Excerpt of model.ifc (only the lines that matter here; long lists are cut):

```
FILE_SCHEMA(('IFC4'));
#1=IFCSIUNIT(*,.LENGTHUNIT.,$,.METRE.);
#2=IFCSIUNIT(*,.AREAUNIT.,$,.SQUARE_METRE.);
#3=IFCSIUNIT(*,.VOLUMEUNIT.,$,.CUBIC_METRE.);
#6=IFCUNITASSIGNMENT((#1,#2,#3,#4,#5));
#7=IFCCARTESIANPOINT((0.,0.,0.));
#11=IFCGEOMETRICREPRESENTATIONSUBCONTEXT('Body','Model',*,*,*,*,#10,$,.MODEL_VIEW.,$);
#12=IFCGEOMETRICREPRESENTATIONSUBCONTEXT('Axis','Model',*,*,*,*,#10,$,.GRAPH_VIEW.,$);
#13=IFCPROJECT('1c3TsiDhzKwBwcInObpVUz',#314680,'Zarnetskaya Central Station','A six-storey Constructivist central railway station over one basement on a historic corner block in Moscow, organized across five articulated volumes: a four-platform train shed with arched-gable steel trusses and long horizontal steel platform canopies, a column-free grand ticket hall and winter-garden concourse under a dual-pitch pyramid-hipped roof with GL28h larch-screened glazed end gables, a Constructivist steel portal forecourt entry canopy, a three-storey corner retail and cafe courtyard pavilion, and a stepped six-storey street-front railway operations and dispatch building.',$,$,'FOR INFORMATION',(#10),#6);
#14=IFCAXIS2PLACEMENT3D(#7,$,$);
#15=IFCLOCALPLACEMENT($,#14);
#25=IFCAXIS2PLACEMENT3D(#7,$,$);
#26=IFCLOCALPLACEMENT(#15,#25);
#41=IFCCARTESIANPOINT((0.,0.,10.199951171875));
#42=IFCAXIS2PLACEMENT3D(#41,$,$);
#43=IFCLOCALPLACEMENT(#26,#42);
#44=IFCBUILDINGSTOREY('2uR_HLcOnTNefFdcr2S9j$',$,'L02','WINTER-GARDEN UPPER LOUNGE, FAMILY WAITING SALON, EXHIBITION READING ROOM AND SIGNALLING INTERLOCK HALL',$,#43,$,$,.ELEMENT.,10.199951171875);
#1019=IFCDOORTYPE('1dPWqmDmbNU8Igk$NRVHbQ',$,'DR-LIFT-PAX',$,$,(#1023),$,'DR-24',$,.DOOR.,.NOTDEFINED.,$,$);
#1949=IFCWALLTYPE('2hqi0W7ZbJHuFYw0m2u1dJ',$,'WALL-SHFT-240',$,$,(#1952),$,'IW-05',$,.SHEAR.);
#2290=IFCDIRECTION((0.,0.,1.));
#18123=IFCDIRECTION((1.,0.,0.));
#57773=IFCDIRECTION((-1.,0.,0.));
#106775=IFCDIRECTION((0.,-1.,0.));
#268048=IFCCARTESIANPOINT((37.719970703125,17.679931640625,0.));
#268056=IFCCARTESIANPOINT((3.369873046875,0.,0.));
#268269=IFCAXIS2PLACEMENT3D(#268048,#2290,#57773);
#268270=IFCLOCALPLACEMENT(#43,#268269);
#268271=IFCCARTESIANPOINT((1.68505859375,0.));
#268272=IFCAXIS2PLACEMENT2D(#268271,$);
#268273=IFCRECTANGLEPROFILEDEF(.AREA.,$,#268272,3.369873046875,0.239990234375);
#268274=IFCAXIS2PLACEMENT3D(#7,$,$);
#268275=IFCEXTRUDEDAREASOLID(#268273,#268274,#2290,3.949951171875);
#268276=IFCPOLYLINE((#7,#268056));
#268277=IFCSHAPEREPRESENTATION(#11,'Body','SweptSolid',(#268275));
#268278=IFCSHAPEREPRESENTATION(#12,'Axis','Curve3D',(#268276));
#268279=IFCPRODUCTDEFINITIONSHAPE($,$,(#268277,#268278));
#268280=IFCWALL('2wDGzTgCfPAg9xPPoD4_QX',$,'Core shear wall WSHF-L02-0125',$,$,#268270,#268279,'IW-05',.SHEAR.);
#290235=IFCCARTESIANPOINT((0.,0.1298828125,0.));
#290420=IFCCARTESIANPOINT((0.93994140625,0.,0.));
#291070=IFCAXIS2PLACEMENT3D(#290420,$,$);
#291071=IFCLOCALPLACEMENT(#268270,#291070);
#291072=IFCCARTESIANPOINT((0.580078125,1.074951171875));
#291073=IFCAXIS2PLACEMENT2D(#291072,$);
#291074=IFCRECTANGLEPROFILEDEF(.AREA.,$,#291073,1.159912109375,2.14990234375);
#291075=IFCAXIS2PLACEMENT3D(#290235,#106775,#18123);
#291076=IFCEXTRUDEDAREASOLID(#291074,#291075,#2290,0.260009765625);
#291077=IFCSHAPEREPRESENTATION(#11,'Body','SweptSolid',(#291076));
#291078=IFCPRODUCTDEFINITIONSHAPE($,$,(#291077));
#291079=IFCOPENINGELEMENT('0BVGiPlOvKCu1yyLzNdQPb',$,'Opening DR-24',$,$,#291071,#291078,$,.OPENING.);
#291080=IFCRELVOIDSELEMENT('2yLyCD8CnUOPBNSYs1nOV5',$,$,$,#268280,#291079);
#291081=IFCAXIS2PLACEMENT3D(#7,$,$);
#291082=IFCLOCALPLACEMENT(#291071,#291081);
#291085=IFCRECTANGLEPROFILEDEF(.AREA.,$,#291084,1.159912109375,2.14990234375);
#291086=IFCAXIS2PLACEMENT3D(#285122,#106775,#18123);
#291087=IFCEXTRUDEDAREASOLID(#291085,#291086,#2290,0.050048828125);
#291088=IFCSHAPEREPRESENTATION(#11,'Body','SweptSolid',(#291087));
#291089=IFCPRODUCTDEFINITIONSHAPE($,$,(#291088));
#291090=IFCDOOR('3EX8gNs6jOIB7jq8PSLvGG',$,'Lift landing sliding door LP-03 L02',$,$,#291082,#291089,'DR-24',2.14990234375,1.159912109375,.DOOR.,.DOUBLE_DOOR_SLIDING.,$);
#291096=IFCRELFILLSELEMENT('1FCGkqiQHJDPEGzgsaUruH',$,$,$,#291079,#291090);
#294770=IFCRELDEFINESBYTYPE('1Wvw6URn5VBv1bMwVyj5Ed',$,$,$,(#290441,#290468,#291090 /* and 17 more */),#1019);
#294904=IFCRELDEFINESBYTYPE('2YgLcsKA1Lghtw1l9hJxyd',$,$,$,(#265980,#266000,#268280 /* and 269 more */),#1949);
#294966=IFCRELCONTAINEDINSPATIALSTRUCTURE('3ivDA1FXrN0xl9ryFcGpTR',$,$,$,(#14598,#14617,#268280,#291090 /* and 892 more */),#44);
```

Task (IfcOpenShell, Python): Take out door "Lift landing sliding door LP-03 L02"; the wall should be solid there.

```python
import ifcopenshell
import ifcopenshell.api.feature
import ifcopenshell.api.root
import ifcopenshell.geom
import ifcopenshell.util.shape

model = ifcopenshell.open("model.ifc")
settings = ifcopenshell.geom.settings()


def volume(element):
    """Net volume in cubic metres, openings subtracted."""
    shape = ifcopenshell.geom.create_shape(settings, element)
    return ifcopenshell.util.shape.get_volume(shape.geometry)


door = model.by_guid("3EX8gNs6jOIB7jq8PSLvGG")
opening = door.FillsVoids[0].RelatingOpeningElement
wall = opening.VoidsElements[0].RelatingBuildingElement
before = volume(wall)

ifcopenshell.api.root.remove_product(model, product=door)
ifcopenshell.api.feature.remove_feature(model, feature=opening)

after = volume(wall)

print(f"wall volume {before:.3f} -> {after:.3f} m3")

model.write("model_rev.ifc")
```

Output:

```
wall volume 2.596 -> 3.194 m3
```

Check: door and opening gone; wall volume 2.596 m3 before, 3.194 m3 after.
